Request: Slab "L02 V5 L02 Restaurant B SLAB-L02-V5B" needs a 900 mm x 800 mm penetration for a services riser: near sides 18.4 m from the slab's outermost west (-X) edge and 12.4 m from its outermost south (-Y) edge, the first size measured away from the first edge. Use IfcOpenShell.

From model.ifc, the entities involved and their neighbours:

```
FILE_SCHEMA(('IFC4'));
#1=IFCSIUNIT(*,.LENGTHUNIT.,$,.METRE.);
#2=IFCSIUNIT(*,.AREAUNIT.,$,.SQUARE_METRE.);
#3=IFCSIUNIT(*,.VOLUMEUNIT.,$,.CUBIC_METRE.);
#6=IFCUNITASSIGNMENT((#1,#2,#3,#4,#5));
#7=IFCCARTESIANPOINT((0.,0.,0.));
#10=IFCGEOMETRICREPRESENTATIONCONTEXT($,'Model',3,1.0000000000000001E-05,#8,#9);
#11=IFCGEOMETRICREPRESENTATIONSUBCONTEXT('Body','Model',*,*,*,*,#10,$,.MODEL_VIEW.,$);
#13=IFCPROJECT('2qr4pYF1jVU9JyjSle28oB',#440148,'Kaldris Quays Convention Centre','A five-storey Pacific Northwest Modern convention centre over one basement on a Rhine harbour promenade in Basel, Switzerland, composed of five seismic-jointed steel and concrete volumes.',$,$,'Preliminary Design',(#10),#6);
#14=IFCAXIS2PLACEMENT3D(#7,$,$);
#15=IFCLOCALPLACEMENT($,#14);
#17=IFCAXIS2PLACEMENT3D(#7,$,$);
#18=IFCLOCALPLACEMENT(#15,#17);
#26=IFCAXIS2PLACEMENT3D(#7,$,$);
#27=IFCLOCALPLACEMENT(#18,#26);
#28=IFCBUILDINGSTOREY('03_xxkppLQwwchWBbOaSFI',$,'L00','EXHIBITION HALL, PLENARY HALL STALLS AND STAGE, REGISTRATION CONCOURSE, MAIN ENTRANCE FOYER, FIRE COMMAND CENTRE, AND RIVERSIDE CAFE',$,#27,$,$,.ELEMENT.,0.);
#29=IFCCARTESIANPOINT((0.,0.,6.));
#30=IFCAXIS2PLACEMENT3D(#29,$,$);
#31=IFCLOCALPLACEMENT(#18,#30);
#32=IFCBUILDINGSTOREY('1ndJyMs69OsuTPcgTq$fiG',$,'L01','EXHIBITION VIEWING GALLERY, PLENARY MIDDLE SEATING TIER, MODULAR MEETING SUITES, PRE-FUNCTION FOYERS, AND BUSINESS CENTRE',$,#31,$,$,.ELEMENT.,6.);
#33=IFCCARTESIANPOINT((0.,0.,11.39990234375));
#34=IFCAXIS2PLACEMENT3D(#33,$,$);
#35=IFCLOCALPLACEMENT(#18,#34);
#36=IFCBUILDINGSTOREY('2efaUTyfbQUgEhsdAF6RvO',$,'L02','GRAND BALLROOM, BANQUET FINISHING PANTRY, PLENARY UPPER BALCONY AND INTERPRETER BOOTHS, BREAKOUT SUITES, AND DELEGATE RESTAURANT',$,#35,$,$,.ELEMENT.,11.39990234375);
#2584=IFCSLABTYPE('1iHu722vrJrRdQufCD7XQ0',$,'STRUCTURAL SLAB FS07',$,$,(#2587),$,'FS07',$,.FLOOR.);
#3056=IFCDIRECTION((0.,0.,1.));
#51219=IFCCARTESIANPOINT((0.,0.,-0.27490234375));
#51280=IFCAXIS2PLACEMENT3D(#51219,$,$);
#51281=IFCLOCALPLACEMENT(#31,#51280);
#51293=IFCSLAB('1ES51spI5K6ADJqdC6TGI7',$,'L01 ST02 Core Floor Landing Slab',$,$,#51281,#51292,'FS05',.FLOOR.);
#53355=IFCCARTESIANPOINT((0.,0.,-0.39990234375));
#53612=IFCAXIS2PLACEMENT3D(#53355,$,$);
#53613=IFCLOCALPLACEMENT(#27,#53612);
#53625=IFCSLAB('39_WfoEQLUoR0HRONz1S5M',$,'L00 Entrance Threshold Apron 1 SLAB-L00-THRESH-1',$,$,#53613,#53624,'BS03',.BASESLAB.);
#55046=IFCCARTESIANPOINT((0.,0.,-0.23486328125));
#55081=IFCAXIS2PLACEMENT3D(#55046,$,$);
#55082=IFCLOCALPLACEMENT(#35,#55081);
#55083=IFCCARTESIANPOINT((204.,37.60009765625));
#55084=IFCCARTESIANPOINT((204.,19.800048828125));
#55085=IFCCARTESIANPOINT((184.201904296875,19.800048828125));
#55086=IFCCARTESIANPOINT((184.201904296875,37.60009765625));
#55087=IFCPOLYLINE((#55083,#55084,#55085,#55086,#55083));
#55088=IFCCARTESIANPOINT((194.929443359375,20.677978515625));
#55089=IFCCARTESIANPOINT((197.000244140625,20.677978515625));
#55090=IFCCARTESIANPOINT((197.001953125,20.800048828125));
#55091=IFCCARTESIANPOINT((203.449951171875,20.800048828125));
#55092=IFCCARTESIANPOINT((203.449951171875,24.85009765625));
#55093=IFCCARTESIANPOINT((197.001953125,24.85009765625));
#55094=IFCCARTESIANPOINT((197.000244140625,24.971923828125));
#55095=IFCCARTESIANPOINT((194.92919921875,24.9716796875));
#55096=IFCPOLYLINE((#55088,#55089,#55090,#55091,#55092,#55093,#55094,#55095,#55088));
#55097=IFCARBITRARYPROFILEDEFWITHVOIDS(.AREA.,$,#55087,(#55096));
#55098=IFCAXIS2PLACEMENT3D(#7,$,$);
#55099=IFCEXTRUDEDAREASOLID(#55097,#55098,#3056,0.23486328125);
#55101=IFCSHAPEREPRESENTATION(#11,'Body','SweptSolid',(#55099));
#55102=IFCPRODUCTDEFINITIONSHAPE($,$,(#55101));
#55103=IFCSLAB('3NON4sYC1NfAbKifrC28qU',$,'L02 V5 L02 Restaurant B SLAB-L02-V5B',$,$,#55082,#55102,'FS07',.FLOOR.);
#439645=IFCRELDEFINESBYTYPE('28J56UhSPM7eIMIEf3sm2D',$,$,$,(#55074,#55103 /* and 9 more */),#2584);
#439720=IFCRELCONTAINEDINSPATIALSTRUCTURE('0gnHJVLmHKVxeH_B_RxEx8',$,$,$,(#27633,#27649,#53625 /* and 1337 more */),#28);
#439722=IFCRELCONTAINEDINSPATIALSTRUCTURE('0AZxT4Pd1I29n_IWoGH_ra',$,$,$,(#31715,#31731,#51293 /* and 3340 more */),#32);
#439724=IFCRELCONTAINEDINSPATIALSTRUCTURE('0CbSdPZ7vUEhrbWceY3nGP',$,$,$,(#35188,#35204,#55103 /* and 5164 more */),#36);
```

```python
import numpy as np
import ifcopenshell
import ifcopenshell.api.feature
import ifcopenshell.api.geometry
import ifcopenshell.api.root
import ifcopenshell.geom
import ifcopenshell.util.placement
import ifcopenshell.util.representation
import ifcopenshell.util.shape
import ifcopenshell.util.unit

model = ifcopenshell.open("model.ifc")
unit_scale = ifcopenshell.util.unit.calculate_unit_scale(model)
settings = ifcopenshell.geom.settings()


def volume(element):
    """Net volume in cubic metres, openings subtracted."""
    shape = ifcopenshell.geom.create_shape(settings, element)
    return ifcopenshell.util.shape.get_volume(shape.geometry)


slab = model.by_guid("3NON4sYC1NfAbKifrC28qU")
before = volume(slab)

# Extent in the slab's own axes, in metres. The edges named are its -X and -Y sides.
slab_shape = ifcopenshell.geom.create_shape(settings, slab)
vertices = ifcopenshell.util.shape.get_vertices(slab_shape.geometry)
x_min, y_min, bottom = vertices.min(axis=0)
top = vertices[:, 2].max()

opening = ifcopenshell.api.root.create_entity(model, ifc_class="IfcOpeningElement", name="Services riser opening", predefined_type="OPENING")
context = ifcopenshell.util.representation.get_context(model, "Model", "Body", "MODEL_VIEW")
width, depth = 0.9, 0.8
outline = [(0.0, 0.0), (width, 0.0), (width, depth), (0.0, depth), (0.0, 0.0)]
# Overshoot both faces by 50 mm so the cut is clean.
shape = ifcopenshell.api.geometry.add_slab_representation(
    model, context=context, depth=top - bottom + 0.1, polyline=outline
)
ifcopenshell.api.geometry.assign_representation(model, product=opening, representation=shape)

matrix = ifcopenshell.util.placement.get_local_placement(slab.ObjectPlacement)
matrix[:, 3] = matrix @ np.append(np.array([x_min + 18.4, y_min + 12.4, bottom - 0.05]) / unit_scale, 1.0)
ifcopenshell.api.geometry.edit_object_placement(model, product=opening, matrix=matrix, is_si=False)
ifcopenshell.api.feature.add_feature(model, feature=opening, element=slab)

after = volume(slab)

print(f"slab volume {before:.3f} -> {after:.3f} m3")

model.write("model-out.ifc")
```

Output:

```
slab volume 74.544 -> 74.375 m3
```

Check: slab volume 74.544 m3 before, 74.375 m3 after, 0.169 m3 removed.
